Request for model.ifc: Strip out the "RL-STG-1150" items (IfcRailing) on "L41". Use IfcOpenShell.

First a look at what the model holds.

```python
import ifcopenshell
import ifcopenshell.util.element

model = ifcopenshell.open("model.ifc")
print(model.schema)
storey = next(s for s in model.by_type("IfcBuildingStorey") if s.Name == "L41")
railings = [e for e in ifcopenshell.util.element.get_decomposition(storey) if e.is_a("IfcRailing")]
seen = {}
for e in railings:
    element_type = ifcopenshell.util.element.get_type(e)
    name = element_type.Name if element_type not in (None, e) else None
    seen[name] = seen.get(name, 0) + 1
for name, count in sorted(seen.items(), key=str):
    print(count, "x", name)
```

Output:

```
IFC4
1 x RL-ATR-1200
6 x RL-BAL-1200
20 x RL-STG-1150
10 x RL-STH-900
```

```python
import ifcopenshell
import ifcopenshell.api.root
import ifcopenshell.util.element

model = ifcopenshell.open("model.ifc")

storey = next(s for s in model.by_type("IfcBuildingStorey") if s.Name == "L41")
railings = [e for e in ifcopenshell.util.element.get_decomposition(storey) if e.is_a("IfcRailing")]
targets = [e for e in railings if (t := ifcopenshell.util.element.get_type(e)) not in (None, e) and t.Name == "RL-STG-1150"]

for e in targets:
    ifcopenshell.api.root.remove_product(model, product=e)
print(len(targets), "removed")

model.write("model_updated.ifc")
```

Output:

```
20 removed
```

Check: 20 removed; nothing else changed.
